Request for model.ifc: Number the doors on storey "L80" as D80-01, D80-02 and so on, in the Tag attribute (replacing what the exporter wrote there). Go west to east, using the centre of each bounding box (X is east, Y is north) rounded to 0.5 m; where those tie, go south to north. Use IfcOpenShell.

First a look at what the model holds.

```python
import ifcopenshell
import ifcopenshell.util.element
import ifcopenshell.util.placement

model = ifcopenshell.open("model.ifc")
print(model.schema)
storey = next(s for s in model.by_type("IfcBuildingStorey") if s.Name == "L80")
doors = [e for e in ifcopenshell.util.element.get_decomposition(storey) if e.is_a("IfcDoor")]
for e in sorted(doors, key=lambda e: e.id()):
    origin = ifcopenshell.util.placement.get_local_placement(e.ObjectPlacement)[:3, 3]
    print(e.id(), e.Tag, e.Name, origin.round(2) + 0.0, sep=" | ")
```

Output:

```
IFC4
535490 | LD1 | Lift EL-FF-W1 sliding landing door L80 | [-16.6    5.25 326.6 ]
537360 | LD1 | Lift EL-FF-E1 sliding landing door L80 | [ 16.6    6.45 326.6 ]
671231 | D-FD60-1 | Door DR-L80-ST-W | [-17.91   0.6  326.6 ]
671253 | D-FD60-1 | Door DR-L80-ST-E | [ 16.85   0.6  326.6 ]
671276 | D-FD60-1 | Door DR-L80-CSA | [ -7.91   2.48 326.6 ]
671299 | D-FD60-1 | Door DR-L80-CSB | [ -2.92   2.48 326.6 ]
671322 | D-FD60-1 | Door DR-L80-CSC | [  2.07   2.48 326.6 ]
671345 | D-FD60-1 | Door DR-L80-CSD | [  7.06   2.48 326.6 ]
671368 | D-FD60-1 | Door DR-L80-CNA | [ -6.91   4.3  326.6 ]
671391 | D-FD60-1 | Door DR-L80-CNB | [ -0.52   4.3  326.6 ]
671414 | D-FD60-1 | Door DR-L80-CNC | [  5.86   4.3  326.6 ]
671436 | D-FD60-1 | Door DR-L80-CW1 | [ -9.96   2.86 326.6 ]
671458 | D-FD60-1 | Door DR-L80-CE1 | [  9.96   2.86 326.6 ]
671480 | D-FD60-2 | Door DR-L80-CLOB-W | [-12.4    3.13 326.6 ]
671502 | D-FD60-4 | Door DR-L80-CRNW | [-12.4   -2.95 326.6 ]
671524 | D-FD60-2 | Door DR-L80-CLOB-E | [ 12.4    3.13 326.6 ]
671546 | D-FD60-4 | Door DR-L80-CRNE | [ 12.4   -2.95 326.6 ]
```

```python
import ifcopenshell
import ifcopenshell.geom
import ifcopenshell.util.element
import ifcopenshell.util.shape

model = ifcopenshell.open("model.ifc")
settings = ifcopenshell.geom.settings()
settings.set("use-world-coords", True)


def centre(element):
    shape = ifcopenshell.geom.create_shape(settings, element)
    return ifcopenshell.util.shape.get_bbox_centroid(shape.geometry)


storey = next(s for s in model.by_type("IfcBuildingStorey") if s.Name == "L80")
doors = [e for e in ifcopenshell.util.element.get_decomposition(storey) if e.is_a("IfcDoor")]

# Insertion points can sit at a corner or the storey origin, so sort by the geometry (in metres).
centres = {e: centre(e) for e in doors}
doors.sort(key=lambda e: (round(centres[e][0] / 0.5), centres[e][1]))

for i, e in enumerate(doors, start=1):
    number = f"D80-{i:02d}"
    e.Tag = number
    print(e.id(), number)

model.write("model_v2.ifc")
```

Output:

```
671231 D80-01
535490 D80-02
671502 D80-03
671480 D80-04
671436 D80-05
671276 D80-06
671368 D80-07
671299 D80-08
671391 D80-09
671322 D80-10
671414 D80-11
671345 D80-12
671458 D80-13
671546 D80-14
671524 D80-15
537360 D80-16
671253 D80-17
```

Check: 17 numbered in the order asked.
